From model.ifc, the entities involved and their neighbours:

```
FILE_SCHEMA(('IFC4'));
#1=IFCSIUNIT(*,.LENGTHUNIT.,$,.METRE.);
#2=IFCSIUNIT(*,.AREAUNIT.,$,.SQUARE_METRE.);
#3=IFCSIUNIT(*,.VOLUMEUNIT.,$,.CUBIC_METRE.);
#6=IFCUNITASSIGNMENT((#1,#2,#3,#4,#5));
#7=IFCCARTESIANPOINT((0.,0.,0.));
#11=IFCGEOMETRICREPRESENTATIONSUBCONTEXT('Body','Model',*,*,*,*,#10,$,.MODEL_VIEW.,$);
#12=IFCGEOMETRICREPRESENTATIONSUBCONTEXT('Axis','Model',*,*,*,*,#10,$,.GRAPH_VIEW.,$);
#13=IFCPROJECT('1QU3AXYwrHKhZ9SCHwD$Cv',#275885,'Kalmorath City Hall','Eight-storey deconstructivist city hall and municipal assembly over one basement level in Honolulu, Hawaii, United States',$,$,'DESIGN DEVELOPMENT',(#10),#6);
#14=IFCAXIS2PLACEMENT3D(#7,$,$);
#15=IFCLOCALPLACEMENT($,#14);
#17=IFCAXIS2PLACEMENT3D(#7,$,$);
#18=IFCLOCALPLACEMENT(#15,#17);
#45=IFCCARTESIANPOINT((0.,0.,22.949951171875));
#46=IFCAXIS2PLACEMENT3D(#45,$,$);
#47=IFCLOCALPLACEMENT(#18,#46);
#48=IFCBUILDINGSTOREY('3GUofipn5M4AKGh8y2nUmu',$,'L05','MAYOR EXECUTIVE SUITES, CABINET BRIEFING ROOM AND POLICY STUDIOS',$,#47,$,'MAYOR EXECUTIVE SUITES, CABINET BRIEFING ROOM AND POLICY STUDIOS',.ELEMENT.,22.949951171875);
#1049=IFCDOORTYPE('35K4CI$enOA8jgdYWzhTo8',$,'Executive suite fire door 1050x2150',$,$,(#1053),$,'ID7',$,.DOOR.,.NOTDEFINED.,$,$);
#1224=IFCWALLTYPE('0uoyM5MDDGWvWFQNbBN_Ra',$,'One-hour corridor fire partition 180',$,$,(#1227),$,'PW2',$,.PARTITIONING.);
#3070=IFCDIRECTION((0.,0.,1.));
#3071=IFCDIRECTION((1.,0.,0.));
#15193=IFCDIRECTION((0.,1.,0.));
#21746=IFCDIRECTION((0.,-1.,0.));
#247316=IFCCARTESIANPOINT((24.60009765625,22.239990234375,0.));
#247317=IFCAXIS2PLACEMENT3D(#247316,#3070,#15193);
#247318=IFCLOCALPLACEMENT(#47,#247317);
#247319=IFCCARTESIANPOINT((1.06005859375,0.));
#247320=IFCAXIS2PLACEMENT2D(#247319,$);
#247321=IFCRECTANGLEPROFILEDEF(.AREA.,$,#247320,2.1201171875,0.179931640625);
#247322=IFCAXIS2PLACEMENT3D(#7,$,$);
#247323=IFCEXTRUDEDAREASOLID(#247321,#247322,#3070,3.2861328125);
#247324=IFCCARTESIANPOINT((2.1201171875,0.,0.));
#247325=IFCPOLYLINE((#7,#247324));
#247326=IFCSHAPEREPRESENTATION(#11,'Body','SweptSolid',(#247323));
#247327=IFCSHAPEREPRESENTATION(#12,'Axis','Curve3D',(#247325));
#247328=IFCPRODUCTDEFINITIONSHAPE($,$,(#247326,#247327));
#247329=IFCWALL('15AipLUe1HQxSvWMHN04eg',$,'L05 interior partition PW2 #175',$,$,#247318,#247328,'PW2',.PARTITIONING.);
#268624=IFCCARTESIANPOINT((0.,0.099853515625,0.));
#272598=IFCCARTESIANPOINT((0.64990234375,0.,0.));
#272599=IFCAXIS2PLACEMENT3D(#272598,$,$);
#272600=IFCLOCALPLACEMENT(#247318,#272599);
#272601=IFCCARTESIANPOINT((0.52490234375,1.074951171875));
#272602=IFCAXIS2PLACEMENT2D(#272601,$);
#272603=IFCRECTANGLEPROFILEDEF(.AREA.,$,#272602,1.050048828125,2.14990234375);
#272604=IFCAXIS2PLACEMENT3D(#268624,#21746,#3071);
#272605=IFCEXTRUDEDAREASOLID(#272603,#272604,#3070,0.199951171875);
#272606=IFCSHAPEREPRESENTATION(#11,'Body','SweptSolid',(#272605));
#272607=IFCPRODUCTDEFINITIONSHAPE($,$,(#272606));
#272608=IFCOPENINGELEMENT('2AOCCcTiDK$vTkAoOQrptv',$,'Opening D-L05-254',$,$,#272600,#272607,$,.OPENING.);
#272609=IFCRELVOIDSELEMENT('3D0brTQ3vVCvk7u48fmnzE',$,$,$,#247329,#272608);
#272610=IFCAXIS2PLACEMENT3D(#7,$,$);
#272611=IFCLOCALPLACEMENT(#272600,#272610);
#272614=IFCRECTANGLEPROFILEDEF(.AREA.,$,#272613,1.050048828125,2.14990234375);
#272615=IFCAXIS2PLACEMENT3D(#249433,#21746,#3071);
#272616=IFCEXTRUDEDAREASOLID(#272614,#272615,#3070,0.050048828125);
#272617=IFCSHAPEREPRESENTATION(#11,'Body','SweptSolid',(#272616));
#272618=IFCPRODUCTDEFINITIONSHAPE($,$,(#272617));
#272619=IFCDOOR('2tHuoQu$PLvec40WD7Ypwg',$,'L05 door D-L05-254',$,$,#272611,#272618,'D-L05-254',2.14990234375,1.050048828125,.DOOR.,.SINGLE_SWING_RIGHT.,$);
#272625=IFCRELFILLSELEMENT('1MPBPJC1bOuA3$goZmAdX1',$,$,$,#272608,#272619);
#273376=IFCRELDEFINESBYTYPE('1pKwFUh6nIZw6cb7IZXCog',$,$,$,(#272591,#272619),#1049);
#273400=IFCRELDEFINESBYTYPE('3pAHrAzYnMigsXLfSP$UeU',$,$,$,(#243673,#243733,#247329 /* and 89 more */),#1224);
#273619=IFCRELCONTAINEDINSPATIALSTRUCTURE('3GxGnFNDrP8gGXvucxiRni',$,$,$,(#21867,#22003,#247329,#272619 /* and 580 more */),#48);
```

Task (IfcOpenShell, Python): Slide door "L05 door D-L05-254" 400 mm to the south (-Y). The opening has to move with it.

```python
import ifcopenshell
import ifcopenshell.api.geometry
import ifcopenshell.util.placement
import ifcopenshell.util.unit

model = ifcopenshell.open("model.ifc")
unit_scale = ifcopenshell.util.unit.calculate_unit_scale(model)

door = model.by_guid("2tHuoQu$PLvec40WD7Ypwg")
opening = door.FillsVoids[0].RelatingOpeningElement
wall = opening.VoidsElements[0].RelatingBuildingElement

wall_matrix = ifcopenshell.util.placement.get_local_placement(wall.ObjectPlacement)
shift = wall_matrix[:3, 0] * -0.4 / unit_scale
before = ifcopenshell.util.placement.get_local_placement(door.ObjectPlacement)[:3, 3].copy()

# The door is placed relative to its opening, so it follows when the opening moves.
matrix = ifcopenshell.util.placement.get_local_placement(opening.ObjectPlacement)
matrix[:3, 3] += shift
ifcopenshell.api.geometry.edit_object_placement(
    model, product=opening, matrix=matrix, is_si=False, should_transform_children=True
)

after = ifcopenshell.util.placement.get_local_placement(door.ObjectPlacement)[:3, 3]
print("door moved by", (after - before).round(3) + 0.0)

model.write("model_v2.ifc")
```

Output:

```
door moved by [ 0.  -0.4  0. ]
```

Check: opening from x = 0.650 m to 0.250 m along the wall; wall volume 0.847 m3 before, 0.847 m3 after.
